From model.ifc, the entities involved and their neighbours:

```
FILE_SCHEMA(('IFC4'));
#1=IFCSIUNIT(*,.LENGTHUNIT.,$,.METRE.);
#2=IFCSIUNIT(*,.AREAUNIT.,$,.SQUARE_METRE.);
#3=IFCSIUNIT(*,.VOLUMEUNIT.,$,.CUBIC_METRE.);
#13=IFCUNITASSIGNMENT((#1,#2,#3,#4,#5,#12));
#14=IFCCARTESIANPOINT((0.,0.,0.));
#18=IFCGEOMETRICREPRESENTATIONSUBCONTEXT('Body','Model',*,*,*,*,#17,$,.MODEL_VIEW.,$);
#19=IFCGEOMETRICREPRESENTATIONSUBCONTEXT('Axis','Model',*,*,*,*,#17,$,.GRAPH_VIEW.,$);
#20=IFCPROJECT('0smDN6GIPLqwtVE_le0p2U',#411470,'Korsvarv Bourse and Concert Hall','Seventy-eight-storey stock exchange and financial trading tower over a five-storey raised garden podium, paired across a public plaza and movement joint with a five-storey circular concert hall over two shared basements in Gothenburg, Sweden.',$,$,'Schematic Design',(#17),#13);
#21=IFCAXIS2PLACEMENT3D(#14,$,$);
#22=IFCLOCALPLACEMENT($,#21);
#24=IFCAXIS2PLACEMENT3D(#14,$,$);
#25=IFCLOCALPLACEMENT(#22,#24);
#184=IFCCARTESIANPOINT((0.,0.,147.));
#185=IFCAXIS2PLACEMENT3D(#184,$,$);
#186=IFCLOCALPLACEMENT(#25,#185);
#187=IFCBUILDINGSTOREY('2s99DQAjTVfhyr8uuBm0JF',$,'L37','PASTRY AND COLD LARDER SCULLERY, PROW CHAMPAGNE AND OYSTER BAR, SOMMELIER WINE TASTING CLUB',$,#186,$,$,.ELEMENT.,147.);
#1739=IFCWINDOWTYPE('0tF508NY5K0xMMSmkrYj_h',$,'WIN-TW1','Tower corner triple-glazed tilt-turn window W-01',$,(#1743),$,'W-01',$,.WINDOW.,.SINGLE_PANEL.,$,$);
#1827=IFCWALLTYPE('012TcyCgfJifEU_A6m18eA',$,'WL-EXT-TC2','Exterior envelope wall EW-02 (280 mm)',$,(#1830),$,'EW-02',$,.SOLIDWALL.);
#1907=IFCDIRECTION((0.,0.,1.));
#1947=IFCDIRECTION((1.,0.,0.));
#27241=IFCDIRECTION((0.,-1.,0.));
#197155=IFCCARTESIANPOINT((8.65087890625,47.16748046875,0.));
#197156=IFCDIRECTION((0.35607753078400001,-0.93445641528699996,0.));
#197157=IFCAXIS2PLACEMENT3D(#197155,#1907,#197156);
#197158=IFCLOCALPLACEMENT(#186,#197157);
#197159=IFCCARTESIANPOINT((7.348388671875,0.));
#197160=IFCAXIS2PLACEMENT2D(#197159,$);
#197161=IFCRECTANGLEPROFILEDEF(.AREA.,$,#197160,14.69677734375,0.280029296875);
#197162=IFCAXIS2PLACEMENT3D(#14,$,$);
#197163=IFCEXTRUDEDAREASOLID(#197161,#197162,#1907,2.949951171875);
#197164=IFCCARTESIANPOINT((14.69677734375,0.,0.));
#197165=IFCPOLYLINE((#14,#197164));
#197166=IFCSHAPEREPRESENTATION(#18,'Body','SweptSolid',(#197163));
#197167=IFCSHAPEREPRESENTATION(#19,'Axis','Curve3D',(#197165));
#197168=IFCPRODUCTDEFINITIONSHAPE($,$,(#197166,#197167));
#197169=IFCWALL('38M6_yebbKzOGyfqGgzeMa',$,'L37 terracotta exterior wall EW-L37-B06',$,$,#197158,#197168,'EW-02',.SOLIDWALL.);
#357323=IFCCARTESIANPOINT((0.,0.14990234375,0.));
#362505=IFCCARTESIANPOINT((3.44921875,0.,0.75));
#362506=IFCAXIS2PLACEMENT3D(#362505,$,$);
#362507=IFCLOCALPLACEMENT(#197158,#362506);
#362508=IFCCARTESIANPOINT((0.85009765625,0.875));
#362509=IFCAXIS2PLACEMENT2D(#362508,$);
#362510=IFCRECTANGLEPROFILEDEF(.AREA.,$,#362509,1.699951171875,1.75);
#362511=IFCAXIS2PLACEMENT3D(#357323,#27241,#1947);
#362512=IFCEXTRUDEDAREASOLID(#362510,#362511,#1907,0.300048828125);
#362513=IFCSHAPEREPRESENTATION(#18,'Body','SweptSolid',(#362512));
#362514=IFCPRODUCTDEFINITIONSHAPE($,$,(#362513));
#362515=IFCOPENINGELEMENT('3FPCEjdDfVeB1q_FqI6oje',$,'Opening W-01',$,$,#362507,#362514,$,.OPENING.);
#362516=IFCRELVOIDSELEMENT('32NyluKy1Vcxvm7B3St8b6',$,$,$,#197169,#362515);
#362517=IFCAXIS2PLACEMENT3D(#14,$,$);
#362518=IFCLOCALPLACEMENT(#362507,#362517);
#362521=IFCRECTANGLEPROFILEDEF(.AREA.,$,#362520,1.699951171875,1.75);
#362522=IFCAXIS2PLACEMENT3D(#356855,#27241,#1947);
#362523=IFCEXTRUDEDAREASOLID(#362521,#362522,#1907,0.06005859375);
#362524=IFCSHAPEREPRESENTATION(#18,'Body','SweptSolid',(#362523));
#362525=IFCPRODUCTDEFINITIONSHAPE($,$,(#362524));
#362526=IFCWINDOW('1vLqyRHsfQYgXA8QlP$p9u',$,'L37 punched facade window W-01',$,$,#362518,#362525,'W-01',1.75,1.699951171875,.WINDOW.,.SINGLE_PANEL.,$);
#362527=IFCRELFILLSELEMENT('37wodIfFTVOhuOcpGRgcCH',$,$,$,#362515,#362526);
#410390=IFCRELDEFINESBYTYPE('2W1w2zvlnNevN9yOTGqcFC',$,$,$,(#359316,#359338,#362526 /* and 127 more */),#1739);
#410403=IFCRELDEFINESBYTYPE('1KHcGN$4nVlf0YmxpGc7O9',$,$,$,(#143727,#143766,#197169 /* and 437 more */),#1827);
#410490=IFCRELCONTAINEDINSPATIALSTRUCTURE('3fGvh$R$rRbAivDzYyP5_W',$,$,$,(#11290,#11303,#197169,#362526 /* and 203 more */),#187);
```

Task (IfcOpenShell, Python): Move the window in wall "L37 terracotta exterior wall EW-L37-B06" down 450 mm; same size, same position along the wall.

```python
import numpy as np
import ifcopenshell
import ifcopenshell.api.geometry
import ifcopenshell.util.placement
import ifcopenshell.util.unit

model = ifcopenshell.open("model.ifc")
unit_scale = ifcopenshell.util.unit.calculate_unit_scale(model)

window = model.by_id(362526)
opening = window.FillsVoids[0].RelatingOpeningElement
dz = -0.45 / unit_scale

shift = np.array([0.0, 0.0, dz])
# The window is placed relative to its opening, so it follows when the opening moves.
matrix = ifcopenshell.util.placement.get_local_placement(opening.ObjectPlacement)
matrix[:3, 3] += shift
ifcopenshell.api.geometry.edit_object_placement(
    model, product=opening, matrix=matrix, is_si=False, should_transform_children=True
)

print(f"moved by {dz * unit_scale:+.3f} m")

model.write("model-out.ifc")
```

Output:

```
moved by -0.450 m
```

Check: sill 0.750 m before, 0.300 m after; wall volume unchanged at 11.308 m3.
